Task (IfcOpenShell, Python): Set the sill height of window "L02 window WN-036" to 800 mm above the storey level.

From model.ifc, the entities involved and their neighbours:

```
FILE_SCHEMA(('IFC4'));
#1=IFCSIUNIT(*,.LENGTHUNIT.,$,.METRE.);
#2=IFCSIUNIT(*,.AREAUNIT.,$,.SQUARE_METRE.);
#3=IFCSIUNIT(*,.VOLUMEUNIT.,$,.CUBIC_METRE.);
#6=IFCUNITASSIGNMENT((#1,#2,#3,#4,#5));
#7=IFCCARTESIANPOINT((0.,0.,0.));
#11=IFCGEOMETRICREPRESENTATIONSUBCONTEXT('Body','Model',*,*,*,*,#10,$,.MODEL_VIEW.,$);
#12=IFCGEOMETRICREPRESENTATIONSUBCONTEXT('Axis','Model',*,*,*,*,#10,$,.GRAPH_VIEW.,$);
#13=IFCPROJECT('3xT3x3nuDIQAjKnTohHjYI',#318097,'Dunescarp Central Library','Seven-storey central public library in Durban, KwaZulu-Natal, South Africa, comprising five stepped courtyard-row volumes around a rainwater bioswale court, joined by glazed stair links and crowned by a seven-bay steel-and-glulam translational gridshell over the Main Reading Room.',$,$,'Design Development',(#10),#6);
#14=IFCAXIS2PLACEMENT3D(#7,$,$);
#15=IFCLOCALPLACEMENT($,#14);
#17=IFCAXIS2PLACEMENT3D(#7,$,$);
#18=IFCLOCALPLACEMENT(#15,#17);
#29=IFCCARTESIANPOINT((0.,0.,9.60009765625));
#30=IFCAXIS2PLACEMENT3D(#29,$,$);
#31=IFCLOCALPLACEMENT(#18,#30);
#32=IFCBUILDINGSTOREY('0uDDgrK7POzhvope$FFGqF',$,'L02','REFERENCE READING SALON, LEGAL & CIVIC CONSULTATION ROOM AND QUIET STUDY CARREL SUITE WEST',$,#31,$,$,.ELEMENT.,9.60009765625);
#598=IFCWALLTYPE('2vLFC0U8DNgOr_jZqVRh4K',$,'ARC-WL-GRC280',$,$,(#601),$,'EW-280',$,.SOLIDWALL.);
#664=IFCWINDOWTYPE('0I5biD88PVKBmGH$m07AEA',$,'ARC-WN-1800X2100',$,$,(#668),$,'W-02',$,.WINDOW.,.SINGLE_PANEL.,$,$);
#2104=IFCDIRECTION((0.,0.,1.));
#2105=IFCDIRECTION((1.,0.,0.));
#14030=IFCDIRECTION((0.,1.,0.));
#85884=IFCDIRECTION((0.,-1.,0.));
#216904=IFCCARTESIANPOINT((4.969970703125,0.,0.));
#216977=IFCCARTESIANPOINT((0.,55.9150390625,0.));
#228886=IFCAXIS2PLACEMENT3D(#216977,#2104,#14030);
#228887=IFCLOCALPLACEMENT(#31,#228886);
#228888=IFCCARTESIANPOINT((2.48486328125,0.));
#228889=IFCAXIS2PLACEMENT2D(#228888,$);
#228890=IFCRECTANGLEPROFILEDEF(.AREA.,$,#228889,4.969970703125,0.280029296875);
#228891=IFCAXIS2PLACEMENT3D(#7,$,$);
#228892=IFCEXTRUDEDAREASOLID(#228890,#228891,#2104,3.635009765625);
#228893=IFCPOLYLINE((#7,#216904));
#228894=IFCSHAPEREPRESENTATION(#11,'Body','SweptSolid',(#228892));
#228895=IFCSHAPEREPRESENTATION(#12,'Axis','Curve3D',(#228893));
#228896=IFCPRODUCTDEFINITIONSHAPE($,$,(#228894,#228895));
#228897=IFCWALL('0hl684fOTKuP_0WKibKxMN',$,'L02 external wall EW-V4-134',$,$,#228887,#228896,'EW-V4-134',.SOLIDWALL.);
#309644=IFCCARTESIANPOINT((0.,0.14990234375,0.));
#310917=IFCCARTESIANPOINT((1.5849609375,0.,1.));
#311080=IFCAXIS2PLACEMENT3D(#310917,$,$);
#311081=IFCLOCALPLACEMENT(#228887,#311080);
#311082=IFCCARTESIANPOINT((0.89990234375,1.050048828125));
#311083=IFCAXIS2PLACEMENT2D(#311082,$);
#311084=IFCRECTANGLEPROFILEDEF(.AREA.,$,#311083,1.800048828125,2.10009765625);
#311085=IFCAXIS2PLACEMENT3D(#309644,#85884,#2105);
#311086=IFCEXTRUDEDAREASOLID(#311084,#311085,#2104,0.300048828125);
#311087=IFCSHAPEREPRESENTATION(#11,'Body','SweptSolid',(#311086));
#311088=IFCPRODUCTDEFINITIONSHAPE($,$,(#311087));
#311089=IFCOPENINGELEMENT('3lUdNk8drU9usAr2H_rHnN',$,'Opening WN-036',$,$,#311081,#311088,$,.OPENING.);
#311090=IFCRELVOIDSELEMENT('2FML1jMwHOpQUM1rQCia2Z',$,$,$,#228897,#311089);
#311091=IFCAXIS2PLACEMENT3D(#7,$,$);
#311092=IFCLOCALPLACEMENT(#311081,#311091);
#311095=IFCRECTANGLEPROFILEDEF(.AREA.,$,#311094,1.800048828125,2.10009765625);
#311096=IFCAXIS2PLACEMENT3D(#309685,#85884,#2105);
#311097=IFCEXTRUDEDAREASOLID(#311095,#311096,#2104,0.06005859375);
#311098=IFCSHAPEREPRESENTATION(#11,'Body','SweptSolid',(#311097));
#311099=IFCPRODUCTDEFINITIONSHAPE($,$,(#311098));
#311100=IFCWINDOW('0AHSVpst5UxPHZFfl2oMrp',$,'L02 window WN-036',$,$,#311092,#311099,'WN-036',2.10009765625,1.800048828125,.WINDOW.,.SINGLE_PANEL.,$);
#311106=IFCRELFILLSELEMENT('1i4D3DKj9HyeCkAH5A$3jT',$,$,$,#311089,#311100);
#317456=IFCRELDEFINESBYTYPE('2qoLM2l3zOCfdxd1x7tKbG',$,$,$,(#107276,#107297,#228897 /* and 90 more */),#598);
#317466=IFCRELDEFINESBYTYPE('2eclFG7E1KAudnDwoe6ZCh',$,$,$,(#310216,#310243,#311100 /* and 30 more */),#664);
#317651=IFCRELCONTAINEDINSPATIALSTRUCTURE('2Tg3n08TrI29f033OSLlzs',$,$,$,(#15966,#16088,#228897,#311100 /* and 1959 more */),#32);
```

```python
import numpy as np
import ifcopenshell
import ifcopenshell.api.geometry
import ifcopenshell.geom
import ifcopenshell.util.element
import ifcopenshell.util.placement
import ifcopenshell.util.shape
import ifcopenshell.util.unit

model = ifcopenshell.open("model.ifc")
unit_scale = ifcopenshell.util.unit.calculate_unit_scale(model)

window = model.by_guid("0AHSVpst5UxPHZFfl2oMrp")
opening = window.FillsVoids[0].RelatingOpeningElement
storey = ifcopenshell.util.element.get_container(window, ifc_class="IfcBuildingStorey")
level = ifcopenshell.util.placement.get_local_placement(storey.ObjectPlacement)[2, 3]

# The opening's origin need not be at the sill, so measure its lowest point.
shape = ifcopenshell.geom.create_shape(ifcopenshell.geom.settings(), opening)
bottom = ifcopenshell.util.shape.get_shape_bottom_elevation(shape, shape.geometry) / unit_scale
dz = level + 0.8 - bottom

shift = np.array([0.0, 0.0, dz])
# The window is placed relative to its opening, so it follows when the opening moves.
matrix = ifcopenshell.util.placement.get_local_placement(opening.ObjectPlacement)
matrix[:3, 3] += shift
ifcopenshell.api.geometry.edit_object_placement(
    model, product=opening, matrix=matrix, is_si=False, should_transform_children=True
)

print(f"moved by {dz * unit_scale:+.3f} m")

model.write("model_v2.ifc")
```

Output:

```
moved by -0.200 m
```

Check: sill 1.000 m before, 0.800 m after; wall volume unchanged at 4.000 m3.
